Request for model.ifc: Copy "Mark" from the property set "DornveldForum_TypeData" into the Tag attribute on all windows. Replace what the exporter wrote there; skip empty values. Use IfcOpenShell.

First a look at what the model holds.

```python
import ifcopenshell
import ifcopenshell.util.element

model = ifcopenshell.open("model.ifc")
print(model.schema)
windows = model.by_type("IfcWindow")
print(len(windows), "windows")
for e in windows[:8]:
    source = ifcopenshell.util.element.get_pset(e, "DornveldForum_TypeData", "Mark")
    target = e.Tag
    print(e.id(), repr(source), repr(target), sep=" | ")
```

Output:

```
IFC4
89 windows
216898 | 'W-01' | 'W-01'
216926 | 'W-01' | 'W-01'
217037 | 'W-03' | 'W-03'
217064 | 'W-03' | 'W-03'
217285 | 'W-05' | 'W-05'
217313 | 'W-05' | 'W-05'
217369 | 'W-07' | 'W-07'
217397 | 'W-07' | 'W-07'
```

```python
import ifcopenshell
import ifcopenshell.util.element

model = ifcopenshell.open("model.ifc")

count = 0
for e in model.by_type("IfcWindow"):
    value = ifcopenshell.util.element.get_pset(e, "DornveldForum_TypeData", "Mark")
    current = e.Tag
    if not value or not value.strip() or current == value:
        continue
    e.Tag = value
    count += 1

print(count, "windows updated")

model.write("model_v2.ifc")
```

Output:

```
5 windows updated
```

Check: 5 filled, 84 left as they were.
